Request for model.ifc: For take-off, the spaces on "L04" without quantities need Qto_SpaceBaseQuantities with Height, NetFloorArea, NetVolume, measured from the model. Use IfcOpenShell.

First a look at what the model holds.

```python
import ifcopenshell
import ifcopenshell.util.element
import ifcopenshell.util.unit

model = ifcopenshell.open("model.ifc")
print(model.schema)
for unit_type in ("LENGTHUNIT", "AREAUNIT", "VOLUMEUNIT"):
    print(unit_type, ifcopenshell.util.unit.calculate_unit_scale(model, unit_type))
storey = next(s for s in model.by_type("IfcBuildingStorey") if s.Name == "L04")
spaces = [e for e in ifcopenshell.util.element.get_decomposition(storey) if e.is_a("IfcSpace")]
for e in sorted(spaces, key=lambda e: e.id()):
    print(e.id(), e.is_a(), e.Name, list(ifcopenshell.util.element.get_psets(e, qtos_only=True)), sep=" | ")
```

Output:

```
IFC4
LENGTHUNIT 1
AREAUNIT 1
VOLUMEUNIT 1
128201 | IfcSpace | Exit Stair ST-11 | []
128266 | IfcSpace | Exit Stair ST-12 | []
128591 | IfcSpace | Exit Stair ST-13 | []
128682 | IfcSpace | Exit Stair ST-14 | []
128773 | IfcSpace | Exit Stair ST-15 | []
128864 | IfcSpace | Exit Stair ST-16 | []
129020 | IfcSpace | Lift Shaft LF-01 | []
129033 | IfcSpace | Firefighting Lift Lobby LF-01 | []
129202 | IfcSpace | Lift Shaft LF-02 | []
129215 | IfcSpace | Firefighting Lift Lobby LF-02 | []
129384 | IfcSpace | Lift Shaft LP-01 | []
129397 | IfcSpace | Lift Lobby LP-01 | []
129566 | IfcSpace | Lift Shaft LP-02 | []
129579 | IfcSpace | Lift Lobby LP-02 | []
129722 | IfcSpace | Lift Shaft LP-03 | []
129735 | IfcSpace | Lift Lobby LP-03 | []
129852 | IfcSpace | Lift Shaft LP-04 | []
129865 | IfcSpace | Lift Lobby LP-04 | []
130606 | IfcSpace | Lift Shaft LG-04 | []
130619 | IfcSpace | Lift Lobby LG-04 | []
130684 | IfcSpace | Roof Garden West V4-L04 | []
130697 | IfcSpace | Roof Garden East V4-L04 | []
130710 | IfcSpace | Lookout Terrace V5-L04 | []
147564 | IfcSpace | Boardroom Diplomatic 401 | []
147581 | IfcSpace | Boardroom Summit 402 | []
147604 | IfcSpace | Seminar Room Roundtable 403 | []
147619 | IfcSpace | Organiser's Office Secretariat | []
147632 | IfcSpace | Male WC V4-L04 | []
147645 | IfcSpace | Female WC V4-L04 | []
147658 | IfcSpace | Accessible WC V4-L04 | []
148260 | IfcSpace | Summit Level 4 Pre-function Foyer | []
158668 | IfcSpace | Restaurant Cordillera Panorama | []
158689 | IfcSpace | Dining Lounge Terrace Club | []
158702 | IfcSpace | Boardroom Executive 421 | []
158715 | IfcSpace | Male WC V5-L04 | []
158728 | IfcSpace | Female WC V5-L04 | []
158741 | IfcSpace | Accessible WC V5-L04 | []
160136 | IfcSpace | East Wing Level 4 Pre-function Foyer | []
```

```python
import ifcopenshell
import ifcopenshell.api.pset
import ifcopenshell.geom
import ifcopenshell.util.element
import ifcopenshell.util.shape
import ifcopenshell.util.unit

model = ifcopenshell.open("model.ifc")
unit_scale = ifcopenshell.util.unit.calculate_unit_scale(model)
area_scale = ifcopenshell.util.unit.calculate_unit_scale(model, "AREAUNIT")
volume_scale = ifcopenshell.util.unit.calculate_unit_scale(model, "VOLUMEUNIT")
settings = ifcopenshell.geom.settings()

storey = next(s for s in model.by_type("IfcBuildingStorey") if s.Name == "L04")
spaces = [e for e in ifcopenshell.util.element.get_decomposition(storey) if e.is_a("IfcSpace")]

for e in sorted(spaces, key=lambda e: e.id()):
    if ifcopenshell.util.element.get_psets(e, qtos_only=True, should_inherit=False):
        continue
    # Geometry comes back in metres, in the element's own axes.
    shape = ifcopenshell.geom.create_shape(settings, e)
    values = {
        "Height": ifcopenshell.util.shape.get_z(shape.geometry) / unit_scale,
        "NetFloorArea": ifcopenshell.util.shape.get_footprint_area(shape.geometry) / area_scale,
        "NetVolume": ifcopenshell.util.shape.get_volume(shape.geometry) / volume_scale,
    }
    qto = ifcopenshell.api.pset.add_qto(model, product=e, name="Qto_SpaceBaseQuantities")
    ifcopenshell.api.pset.edit_qto(model, qto=qto, properties=values)
    print(e.id(), {k: round(v, 3) for k, v in values.items()})

model.write("model-out.ifc")
```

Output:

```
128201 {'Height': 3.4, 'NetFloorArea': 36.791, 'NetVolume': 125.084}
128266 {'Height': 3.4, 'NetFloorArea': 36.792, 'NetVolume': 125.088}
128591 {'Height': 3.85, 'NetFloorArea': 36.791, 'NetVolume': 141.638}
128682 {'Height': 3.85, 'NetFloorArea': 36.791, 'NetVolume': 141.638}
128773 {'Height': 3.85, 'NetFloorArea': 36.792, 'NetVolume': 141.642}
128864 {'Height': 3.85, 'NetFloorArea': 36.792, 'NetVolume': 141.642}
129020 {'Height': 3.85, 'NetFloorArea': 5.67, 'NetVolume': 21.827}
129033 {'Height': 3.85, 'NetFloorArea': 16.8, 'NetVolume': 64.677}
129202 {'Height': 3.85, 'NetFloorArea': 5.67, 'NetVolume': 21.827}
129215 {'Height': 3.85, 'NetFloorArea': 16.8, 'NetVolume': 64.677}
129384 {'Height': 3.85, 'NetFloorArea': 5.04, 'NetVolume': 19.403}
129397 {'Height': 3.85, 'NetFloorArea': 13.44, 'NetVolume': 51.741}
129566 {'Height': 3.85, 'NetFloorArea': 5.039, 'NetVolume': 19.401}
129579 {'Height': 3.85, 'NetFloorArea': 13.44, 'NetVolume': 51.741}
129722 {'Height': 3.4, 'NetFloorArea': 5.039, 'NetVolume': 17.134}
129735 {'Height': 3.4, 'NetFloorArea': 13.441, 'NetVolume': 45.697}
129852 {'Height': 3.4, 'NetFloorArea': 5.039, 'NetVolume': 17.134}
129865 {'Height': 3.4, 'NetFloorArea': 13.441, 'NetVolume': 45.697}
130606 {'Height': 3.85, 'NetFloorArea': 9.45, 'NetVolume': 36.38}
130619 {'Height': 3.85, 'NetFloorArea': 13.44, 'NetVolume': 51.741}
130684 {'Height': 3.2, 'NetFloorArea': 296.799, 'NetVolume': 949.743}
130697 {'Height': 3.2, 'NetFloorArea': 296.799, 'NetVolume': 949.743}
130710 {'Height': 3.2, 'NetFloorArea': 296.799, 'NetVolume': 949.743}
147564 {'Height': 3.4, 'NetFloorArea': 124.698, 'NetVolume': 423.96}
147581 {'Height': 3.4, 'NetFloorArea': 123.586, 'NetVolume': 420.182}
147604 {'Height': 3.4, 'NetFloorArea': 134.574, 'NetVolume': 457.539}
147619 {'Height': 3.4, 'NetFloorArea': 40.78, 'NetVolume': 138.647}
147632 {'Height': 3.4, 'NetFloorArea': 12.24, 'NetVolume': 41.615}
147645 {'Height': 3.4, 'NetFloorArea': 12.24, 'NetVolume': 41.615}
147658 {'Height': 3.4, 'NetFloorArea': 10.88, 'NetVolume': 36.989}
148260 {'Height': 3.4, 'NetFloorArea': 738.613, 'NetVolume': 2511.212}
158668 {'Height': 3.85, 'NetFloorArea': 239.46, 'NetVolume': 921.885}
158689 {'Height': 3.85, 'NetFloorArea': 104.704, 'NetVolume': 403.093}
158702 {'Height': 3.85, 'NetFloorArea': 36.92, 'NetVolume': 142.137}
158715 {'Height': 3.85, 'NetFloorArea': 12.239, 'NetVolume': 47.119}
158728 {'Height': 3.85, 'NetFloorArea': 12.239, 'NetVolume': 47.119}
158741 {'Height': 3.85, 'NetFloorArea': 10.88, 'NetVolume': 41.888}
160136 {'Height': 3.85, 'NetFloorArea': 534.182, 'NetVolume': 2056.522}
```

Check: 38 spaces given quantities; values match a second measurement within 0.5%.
